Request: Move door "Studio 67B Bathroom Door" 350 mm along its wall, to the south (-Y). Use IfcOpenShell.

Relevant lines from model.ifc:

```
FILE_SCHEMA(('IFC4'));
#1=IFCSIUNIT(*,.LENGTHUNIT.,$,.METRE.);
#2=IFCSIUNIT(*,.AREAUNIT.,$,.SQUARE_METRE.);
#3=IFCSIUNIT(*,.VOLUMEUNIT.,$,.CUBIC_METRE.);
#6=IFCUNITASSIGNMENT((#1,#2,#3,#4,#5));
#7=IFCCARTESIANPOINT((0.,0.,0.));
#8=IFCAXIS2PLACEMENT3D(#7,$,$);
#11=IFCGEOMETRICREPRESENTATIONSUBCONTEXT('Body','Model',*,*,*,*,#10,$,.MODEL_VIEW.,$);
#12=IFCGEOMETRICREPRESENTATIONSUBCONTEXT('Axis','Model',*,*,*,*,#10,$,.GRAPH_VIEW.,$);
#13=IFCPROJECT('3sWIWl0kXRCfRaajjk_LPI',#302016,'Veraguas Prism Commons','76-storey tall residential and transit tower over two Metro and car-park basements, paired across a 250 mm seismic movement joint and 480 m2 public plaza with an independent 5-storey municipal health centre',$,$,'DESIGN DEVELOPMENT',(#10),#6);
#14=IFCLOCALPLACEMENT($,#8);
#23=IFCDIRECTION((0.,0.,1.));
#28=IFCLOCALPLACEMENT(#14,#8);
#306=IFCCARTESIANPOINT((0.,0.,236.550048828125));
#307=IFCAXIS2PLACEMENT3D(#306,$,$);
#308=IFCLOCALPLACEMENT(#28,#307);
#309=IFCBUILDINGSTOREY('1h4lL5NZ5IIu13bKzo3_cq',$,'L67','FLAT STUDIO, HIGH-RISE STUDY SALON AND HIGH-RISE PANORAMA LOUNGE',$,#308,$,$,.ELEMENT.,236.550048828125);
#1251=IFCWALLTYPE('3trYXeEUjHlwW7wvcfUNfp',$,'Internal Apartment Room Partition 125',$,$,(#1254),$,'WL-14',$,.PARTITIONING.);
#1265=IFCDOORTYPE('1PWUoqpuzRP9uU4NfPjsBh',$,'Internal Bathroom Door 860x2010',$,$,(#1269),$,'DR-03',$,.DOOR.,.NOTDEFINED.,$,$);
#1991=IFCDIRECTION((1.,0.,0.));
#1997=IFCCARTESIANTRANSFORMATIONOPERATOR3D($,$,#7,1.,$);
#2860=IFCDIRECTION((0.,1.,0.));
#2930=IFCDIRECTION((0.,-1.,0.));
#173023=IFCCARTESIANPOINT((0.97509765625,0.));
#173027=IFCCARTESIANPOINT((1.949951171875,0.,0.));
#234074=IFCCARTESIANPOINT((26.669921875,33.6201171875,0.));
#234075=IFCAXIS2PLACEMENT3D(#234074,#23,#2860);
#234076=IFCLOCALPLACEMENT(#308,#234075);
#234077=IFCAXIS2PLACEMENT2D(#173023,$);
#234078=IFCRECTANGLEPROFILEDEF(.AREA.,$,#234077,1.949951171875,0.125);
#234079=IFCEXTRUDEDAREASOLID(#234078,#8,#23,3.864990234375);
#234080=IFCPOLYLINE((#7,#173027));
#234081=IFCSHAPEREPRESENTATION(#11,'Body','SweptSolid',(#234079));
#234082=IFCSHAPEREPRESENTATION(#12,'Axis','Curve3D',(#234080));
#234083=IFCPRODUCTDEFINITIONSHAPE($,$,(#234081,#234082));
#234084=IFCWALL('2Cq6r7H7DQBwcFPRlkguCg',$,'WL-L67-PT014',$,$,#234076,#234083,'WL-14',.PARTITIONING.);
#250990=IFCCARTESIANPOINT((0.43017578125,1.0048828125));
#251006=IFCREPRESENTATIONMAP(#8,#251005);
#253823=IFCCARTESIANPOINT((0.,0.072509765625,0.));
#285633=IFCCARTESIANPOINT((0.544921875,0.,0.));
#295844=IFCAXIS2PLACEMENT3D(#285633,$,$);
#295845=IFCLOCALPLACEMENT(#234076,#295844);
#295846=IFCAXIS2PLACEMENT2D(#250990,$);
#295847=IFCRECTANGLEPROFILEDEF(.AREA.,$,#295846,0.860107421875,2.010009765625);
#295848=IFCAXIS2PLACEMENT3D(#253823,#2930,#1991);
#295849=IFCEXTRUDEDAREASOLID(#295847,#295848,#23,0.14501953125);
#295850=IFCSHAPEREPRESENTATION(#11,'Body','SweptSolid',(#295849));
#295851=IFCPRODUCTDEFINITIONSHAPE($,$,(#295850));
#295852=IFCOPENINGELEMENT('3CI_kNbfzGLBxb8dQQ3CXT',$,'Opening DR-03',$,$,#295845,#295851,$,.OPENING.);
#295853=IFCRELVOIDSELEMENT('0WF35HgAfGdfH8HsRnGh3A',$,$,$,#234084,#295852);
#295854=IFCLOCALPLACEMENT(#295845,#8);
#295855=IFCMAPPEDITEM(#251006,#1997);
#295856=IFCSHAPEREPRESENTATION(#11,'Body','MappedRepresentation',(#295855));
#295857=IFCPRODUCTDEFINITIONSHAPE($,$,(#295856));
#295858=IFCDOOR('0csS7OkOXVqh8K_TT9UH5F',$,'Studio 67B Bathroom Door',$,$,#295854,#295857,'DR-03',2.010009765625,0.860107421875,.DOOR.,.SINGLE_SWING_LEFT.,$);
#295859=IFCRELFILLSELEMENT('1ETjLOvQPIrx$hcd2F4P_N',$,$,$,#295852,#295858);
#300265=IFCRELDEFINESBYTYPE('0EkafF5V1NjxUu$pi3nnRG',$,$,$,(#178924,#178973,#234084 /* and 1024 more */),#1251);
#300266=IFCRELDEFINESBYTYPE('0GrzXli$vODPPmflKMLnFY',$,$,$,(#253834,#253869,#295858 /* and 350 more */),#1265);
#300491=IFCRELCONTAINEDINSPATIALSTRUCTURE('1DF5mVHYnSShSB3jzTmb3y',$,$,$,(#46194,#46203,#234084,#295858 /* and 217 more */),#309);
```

```python
import ifcopenshell
import ifcopenshell.api.geometry
import ifcopenshell.util.placement
import ifcopenshell.util.unit

model = ifcopenshell.open("model.ifc")
unit_scale = ifcopenshell.util.unit.calculate_unit_scale(model)

door = model.by_guid("0csS7OkOXVqh8K_TT9UH5F")
opening = door.FillsVoids[0].RelatingOpeningElement
wall = opening.VoidsElements[0].RelatingBuildingElement

wall_matrix = ifcopenshell.util.placement.get_local_placement(wall.ObjectPlacement)
shift = wall_matrix[:3, 0] * -0.35 / unit_scale
before = ifcopenshell.util.placement.get_local_placement(door.ObjectPlacement)[:3, 3].copy()

# The door is placed relative to its opening, so it follows when the opening moves.
matrix = ifcopenshell.util.placement.get_local_placement(opening.ObjectPlacement)
matrix[:3, 3] += shift
ifcopenshell.api.geometry.edit_object_placement(
    model, product=opening, matrix=matrix, is_si=False, should_transform_children=True
)

after = ifcopenshell.util.placement.get_local_placement(door.ObjectPlacement)[:3, 3]
print("door moved by", (after - before).round(3) + 0.0)

model.write("model_rev.ifc")
```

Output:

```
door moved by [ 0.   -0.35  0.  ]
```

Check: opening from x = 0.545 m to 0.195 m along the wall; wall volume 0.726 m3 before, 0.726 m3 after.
